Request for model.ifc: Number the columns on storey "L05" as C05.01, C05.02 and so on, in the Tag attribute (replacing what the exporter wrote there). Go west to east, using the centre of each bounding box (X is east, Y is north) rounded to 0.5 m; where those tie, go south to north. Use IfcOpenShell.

First a look at what the model holds.

```python
import ifcopenshell
import ifcopenshell.util.element
import ifcopenshell.util.placement

model = ifcopenshell.open("model.ifc")
print(model.schema)
storey = next(s for s in model.by_type("IfcBuildingStorey") if s.Name == "L05")
columns = [e for e in ifcopenshell.util.element.get_decomposition(storey) if e.is_a("IfcColumn")]
for e in sorted(columns, key=lambda e: e.id()):
    origin = ifcopenshell.util.placement.get_local_placement(e.ObjectPlacement)[:3, 3]
    print(e.id(), e.Tag, e.Name, origin.round(2) + 0.0, sep=" | ")
```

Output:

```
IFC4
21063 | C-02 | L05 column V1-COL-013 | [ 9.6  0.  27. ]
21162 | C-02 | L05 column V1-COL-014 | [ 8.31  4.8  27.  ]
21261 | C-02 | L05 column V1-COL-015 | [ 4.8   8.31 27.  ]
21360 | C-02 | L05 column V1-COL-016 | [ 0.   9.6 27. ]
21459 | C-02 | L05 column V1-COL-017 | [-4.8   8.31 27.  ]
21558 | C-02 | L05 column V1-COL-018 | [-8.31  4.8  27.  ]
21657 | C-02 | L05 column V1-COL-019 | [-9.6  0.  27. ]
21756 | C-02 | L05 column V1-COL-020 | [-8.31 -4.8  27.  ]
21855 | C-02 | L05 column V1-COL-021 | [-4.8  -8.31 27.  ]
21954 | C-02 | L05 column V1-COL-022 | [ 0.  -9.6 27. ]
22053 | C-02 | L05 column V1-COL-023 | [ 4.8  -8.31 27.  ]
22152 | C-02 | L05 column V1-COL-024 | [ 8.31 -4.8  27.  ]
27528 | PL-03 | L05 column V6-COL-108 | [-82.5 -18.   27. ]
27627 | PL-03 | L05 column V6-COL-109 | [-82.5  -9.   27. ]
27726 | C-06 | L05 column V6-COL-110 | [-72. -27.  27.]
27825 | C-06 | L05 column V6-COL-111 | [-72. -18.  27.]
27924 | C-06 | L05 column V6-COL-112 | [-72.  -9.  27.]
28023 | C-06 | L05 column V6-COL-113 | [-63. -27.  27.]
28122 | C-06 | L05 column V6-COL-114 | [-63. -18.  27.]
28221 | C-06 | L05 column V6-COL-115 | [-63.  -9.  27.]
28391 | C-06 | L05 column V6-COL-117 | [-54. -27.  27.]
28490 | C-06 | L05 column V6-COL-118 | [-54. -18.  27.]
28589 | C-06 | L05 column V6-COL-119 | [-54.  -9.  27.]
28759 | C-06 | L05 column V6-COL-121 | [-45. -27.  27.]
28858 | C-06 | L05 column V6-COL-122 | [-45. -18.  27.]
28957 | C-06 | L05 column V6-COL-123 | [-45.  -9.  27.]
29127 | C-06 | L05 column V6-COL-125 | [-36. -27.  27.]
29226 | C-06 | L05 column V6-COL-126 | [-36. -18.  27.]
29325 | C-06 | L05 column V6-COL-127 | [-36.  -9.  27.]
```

```python
import ifcopenshell
import ifcopenshell.geom
import ifcopenshell.util.element
import ifcopenshell.util.shape

model = ifcopenshell.open("model.ifc")
settings = ifcopenshell.geom.settings()
settings.set("use-world-coords", True)


def centre(element):
    shape = ifcopenshell.geom.create_shape(settings, element)
    return ifcopenshell.util.shape.get_bbox_centroid(shape.geometry)


storey = next(s for s in model.by_type("IfcBuildingStorey") if s.Name == "L05")
columns = [e for e in ifcopenshell.util.element.get_decomposition(storey) if e.is_a("IfcColumn")]

# Insertion points can sit at a corner or the storey origin, so sort by the geometry (in metres).
centres = {e: centre(e) for e in columns}
columns.sort(key=lambda e: (round(centres[e][0] / 0.5), centres[e][1]))

for i, e in enumerate(columns, start=1):
    number = f"C05.{i:02d}"
    e.Tag = number
    print(e.id(), number)

model.write("model_rev.ifc")
```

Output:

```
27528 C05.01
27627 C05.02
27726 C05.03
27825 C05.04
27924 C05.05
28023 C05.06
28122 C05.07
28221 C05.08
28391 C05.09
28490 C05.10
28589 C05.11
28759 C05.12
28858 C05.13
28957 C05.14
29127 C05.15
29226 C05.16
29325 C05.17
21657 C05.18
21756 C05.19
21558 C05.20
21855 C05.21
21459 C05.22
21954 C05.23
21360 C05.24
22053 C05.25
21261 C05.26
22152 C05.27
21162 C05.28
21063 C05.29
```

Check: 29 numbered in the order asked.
